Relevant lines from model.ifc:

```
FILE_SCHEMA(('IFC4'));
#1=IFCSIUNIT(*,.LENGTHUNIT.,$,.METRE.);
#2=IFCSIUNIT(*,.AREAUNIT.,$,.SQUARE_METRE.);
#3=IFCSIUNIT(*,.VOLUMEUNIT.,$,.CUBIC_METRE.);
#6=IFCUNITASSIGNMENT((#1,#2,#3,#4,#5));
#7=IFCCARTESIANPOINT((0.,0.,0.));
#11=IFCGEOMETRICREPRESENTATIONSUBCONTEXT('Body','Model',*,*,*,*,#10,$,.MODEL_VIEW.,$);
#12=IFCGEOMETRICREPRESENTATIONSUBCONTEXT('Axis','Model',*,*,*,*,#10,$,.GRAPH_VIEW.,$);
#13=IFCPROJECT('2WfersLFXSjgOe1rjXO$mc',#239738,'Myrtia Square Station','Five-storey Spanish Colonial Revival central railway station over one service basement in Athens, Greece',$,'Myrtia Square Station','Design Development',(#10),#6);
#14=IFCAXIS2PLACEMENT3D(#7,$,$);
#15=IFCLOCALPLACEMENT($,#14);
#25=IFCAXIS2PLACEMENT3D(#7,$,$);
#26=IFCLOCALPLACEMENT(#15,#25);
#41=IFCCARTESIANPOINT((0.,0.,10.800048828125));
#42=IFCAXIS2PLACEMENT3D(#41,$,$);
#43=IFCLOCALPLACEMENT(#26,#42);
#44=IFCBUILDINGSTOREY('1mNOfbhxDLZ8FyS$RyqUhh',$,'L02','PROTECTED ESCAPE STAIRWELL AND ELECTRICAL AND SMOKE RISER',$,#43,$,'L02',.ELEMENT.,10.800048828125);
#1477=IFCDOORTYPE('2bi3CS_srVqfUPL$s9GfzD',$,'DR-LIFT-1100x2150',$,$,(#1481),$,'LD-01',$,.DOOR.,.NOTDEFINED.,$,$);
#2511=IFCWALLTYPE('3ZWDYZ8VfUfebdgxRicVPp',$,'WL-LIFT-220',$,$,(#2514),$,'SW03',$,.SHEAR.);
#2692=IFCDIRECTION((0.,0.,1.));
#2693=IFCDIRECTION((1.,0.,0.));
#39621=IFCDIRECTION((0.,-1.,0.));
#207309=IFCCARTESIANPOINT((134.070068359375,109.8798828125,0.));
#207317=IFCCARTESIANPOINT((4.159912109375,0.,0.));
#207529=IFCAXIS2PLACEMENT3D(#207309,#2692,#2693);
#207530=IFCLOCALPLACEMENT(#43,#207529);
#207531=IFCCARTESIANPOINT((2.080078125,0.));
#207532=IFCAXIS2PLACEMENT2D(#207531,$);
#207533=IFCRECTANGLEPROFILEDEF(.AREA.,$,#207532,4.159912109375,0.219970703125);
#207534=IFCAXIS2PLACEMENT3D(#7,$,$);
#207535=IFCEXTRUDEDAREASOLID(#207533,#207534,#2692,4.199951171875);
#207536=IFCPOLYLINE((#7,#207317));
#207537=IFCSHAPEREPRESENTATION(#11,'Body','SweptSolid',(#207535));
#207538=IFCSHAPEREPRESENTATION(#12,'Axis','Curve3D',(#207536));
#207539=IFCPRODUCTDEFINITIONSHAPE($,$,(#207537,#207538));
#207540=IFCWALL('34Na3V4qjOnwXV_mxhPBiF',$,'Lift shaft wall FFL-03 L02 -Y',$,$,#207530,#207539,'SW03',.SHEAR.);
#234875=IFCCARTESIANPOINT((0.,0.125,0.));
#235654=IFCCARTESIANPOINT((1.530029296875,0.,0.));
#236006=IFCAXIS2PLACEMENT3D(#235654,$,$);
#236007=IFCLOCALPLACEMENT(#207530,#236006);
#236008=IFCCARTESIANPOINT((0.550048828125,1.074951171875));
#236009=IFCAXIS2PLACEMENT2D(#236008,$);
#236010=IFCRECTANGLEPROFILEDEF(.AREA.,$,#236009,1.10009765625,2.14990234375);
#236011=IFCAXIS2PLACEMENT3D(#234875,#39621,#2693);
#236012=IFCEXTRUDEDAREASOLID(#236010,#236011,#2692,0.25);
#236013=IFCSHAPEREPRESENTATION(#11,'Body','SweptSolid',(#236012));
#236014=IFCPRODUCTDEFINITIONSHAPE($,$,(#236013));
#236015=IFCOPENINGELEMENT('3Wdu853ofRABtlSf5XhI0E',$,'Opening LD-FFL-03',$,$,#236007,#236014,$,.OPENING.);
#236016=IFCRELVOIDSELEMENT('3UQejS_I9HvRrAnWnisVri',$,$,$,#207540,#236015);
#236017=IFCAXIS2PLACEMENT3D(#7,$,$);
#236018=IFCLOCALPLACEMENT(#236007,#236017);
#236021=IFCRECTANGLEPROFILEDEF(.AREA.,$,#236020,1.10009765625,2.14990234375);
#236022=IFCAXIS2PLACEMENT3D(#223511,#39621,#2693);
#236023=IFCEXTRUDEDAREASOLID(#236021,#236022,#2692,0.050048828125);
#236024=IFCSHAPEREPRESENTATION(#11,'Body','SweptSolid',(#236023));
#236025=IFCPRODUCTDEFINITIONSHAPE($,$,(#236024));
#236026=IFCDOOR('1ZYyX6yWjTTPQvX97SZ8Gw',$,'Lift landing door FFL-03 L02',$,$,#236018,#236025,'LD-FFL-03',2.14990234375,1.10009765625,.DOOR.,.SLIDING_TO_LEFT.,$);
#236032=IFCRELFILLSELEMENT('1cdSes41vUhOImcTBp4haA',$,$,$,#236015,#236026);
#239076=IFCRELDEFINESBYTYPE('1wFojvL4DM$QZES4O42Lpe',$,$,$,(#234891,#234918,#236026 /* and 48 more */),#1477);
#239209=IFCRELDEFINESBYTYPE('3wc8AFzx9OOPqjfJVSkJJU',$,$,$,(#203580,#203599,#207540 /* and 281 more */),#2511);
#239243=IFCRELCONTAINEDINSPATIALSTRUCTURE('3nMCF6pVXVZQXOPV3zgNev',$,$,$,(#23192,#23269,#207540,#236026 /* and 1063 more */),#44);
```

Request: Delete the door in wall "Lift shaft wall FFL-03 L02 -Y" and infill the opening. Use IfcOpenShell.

```python
import ifcopenshell
import ifcopenshell.api.feature
import ifcopenshell.api.root
import ifcopenshell.geom
import ifcopenshell.util.shape

model = ifcopenshell.open("model.ifc")
settings = ifcopenshell.geom.settings()


def volume(element):
    """Net volume in cubic metres, openings subtracted."""
    shape = ifcopenshell.geom.create_shape(settings, element)
    return ifcopenshell.util.shape.get_volume(shape.geometry)


door = model.by_guid("1ZYyX6yWjTTPQvX97SZ8Gw")
opening = door.FillsVoids[0].RelatingOpeningElement
wall = opening.VoidsElements[0].RelatingBuildingElement
before = volume(wall)

ifcopenshell.api.root.remove_product(model, product=door)
ifcopenshell.api.feature.remove_feature(model, feature=opening)

after = volume(wall)

print(f"wall volume {before:.3f} -> {after:.3f} m3")

model.write("model_v2.ifc")
```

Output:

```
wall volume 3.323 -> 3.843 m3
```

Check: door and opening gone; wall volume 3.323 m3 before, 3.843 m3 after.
